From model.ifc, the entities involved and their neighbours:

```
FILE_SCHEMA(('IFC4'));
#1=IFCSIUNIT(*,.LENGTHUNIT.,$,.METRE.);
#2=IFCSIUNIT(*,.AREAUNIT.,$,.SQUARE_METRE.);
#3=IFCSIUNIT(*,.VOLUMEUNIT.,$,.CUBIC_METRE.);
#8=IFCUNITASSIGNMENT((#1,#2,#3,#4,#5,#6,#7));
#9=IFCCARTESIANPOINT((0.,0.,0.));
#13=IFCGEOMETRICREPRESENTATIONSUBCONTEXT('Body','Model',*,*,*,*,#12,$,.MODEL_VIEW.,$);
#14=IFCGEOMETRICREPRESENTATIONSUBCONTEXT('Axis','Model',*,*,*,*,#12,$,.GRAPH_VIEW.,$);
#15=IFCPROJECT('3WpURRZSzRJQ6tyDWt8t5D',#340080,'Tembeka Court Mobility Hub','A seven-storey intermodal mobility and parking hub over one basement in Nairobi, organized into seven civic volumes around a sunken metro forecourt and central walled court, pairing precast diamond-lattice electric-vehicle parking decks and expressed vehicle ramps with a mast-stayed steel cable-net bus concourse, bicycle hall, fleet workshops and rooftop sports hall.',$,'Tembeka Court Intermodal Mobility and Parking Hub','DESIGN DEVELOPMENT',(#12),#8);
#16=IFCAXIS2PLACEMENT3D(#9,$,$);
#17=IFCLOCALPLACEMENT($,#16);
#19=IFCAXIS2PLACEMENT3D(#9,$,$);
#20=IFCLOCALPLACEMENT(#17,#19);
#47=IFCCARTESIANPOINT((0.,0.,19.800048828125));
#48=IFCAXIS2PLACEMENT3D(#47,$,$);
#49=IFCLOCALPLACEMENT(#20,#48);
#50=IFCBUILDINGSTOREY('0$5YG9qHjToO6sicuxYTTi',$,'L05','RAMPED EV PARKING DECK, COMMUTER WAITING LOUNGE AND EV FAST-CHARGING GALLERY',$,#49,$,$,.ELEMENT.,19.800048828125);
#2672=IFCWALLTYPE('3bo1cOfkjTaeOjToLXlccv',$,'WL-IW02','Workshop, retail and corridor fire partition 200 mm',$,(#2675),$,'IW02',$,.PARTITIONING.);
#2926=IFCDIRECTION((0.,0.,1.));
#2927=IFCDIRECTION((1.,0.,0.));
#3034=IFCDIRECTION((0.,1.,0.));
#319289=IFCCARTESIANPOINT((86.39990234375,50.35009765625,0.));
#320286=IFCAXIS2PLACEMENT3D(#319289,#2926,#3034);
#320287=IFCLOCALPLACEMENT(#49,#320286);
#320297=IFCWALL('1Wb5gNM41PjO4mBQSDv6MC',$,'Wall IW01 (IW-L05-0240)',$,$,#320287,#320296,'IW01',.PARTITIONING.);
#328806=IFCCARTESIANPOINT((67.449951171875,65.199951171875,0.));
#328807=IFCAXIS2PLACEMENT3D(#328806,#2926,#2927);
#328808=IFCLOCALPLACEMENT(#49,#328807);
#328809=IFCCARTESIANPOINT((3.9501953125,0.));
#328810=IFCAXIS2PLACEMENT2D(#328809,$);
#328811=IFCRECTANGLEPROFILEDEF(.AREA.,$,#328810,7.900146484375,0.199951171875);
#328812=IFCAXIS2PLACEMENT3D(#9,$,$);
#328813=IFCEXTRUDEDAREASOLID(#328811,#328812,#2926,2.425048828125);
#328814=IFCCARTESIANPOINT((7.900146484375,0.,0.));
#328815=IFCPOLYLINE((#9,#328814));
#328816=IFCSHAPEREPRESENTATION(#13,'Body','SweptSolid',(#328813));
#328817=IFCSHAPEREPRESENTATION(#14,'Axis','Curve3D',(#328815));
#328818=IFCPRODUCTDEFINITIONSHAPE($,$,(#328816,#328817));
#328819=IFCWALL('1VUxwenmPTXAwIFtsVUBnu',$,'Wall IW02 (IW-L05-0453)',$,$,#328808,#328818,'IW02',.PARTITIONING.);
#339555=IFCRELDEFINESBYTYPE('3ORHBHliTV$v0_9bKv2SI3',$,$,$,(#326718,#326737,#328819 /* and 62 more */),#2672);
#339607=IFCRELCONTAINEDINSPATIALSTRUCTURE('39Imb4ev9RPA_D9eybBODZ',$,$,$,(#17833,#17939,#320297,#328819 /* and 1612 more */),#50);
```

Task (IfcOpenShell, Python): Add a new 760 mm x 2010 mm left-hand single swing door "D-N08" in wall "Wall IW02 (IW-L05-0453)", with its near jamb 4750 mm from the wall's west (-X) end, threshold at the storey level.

```python
import numpy as np
import ifcopenshell
import ifcopenshell.api.feature
import ifcopenshell.api.geometry
import ifcopenshell.api.root
import ifcopenshell.api.spatial
import ifcopenshell.geom
import ifcopenshell.util.element
import ifcopenshell.util.placement
import ifcopenshell.util.representation
import ifcopenshell.util.shape
import ifcopenshell.util.unit

model = ifcopenshell.open("model.ifc")
unit_scale = ifcopenshell.util.unit.calculate_unit_scale(model)
settings = ifcopenshell.geom.settings()


def volume(element):
    """Net volume in cubic metres, openings subtracted."""
    shape = ifcopenshell.geom.create_shape(settings, element)
    return ifcopenshell.util.shape.get_volume(shape.geometry)


wall = model.by_guid("1VUxwenmPTXAwIFtsVUBnu")
storey = ifcopenshell.util.element.get_container(wall, ifc_class="IfcBuildingStorey")
context = ifcopenshell.util.representation.get_context(model, "Model", "Body", "MODEL_VIEW")
before = volume(wall)

width, height, from_end, sill = 0.76, 2.01, 4.75, 0.0  # metres

# The wall runs along its own X axis, and the end named is its -X end.
wall_shape = ifcopenshell.geom.create_shape(settings, wall)
x, y, z = ifcopenshell.util.shape.get_vertices(wall_shape.geometry).T
start = x.min() + from_end
face, thickness = float(y.min()), float(y.max() - y.min())
wall_matrix = ifcopenshell.util.placement.get_local_placement(wall.ObjectPlacement)
level = ifcopenshell.util.placement.get_local_placement(storey.ObjectPlacement)[2, 3]


def in_wall(x, y):
    """Placement at x, y metres in the wall's axes, at sill height."""
    matrix = wall_matrix.copy()
    matrix[:, 3] = wall_matrix @ np.array([x / unit_scale, y / unit_scale, 0.0, 1.0])
    matrix[2, 3] = level + sill / unit_scale
    return matrix


# Opening: a box that overshoots both wall faces by 50 mm.
opening = ifcopenshell.api.root.create_entity(model, ifc_class="IfcOpeningElement", predefined_type="OPENING")
box = ifcopenshell.api.geometry.add_wall_representation(
    model, context=context, length=width, height=height, thickness=thickness + 0.1
)
ifcopenshell.api.geometry.assign_representation(model, product=opening, representation=box)
ifcopenshell.api.geometry.edit_object_placement(model, product=opening, matrix=in_wall(start, face - 0.05), is_si=False)
ifcopenshell.api.feature.add_feature(model, feature=opening, element=wall)

door = ifcopenshell.api.root.create_entity(model, ifc_class="IfcDoor", name="D-N08", predefined_type="DOOR")
door.OverallWidth, door.OverallHeight = width / unit_scale, height / unit_scale
door.OperationType = "SINGLE_SWING_LEFT"
body = ifcopenshell.api.geometry.add_door_representation(
    model,
    context=context,
    overall_width=door.OverallWidth,
    overall_height=door.OverallHeight,
    operation_type="SINGLE_SWING_LEFT",
    lining_properties={"LiningDepth": thickness / unit_scale, "ThresholdDepth": thickness / unit_scale},
)
ifcopenshell.api.geometry.assign_representation(model, product=door, representation=body)
ifcopenshell.api.spatial.assign_container(model, products=[door], relating_structure=storey)
ifcopenshell.api.feature.add_filling(model, opening=opening, element=door)

# The lining spans the wall, so the door starts at the wall face.
ifcopenshell.api.geometry.edit_object_placement(model, product=door, matrix=in_wall(start, face), is_si=False)

after = volume(wall)

print(f"wall volume {before:.3f} -> {after:.3f} m3")

model.write("model_rev.ifc")
```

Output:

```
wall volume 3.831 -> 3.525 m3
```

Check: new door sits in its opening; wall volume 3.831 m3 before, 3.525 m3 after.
